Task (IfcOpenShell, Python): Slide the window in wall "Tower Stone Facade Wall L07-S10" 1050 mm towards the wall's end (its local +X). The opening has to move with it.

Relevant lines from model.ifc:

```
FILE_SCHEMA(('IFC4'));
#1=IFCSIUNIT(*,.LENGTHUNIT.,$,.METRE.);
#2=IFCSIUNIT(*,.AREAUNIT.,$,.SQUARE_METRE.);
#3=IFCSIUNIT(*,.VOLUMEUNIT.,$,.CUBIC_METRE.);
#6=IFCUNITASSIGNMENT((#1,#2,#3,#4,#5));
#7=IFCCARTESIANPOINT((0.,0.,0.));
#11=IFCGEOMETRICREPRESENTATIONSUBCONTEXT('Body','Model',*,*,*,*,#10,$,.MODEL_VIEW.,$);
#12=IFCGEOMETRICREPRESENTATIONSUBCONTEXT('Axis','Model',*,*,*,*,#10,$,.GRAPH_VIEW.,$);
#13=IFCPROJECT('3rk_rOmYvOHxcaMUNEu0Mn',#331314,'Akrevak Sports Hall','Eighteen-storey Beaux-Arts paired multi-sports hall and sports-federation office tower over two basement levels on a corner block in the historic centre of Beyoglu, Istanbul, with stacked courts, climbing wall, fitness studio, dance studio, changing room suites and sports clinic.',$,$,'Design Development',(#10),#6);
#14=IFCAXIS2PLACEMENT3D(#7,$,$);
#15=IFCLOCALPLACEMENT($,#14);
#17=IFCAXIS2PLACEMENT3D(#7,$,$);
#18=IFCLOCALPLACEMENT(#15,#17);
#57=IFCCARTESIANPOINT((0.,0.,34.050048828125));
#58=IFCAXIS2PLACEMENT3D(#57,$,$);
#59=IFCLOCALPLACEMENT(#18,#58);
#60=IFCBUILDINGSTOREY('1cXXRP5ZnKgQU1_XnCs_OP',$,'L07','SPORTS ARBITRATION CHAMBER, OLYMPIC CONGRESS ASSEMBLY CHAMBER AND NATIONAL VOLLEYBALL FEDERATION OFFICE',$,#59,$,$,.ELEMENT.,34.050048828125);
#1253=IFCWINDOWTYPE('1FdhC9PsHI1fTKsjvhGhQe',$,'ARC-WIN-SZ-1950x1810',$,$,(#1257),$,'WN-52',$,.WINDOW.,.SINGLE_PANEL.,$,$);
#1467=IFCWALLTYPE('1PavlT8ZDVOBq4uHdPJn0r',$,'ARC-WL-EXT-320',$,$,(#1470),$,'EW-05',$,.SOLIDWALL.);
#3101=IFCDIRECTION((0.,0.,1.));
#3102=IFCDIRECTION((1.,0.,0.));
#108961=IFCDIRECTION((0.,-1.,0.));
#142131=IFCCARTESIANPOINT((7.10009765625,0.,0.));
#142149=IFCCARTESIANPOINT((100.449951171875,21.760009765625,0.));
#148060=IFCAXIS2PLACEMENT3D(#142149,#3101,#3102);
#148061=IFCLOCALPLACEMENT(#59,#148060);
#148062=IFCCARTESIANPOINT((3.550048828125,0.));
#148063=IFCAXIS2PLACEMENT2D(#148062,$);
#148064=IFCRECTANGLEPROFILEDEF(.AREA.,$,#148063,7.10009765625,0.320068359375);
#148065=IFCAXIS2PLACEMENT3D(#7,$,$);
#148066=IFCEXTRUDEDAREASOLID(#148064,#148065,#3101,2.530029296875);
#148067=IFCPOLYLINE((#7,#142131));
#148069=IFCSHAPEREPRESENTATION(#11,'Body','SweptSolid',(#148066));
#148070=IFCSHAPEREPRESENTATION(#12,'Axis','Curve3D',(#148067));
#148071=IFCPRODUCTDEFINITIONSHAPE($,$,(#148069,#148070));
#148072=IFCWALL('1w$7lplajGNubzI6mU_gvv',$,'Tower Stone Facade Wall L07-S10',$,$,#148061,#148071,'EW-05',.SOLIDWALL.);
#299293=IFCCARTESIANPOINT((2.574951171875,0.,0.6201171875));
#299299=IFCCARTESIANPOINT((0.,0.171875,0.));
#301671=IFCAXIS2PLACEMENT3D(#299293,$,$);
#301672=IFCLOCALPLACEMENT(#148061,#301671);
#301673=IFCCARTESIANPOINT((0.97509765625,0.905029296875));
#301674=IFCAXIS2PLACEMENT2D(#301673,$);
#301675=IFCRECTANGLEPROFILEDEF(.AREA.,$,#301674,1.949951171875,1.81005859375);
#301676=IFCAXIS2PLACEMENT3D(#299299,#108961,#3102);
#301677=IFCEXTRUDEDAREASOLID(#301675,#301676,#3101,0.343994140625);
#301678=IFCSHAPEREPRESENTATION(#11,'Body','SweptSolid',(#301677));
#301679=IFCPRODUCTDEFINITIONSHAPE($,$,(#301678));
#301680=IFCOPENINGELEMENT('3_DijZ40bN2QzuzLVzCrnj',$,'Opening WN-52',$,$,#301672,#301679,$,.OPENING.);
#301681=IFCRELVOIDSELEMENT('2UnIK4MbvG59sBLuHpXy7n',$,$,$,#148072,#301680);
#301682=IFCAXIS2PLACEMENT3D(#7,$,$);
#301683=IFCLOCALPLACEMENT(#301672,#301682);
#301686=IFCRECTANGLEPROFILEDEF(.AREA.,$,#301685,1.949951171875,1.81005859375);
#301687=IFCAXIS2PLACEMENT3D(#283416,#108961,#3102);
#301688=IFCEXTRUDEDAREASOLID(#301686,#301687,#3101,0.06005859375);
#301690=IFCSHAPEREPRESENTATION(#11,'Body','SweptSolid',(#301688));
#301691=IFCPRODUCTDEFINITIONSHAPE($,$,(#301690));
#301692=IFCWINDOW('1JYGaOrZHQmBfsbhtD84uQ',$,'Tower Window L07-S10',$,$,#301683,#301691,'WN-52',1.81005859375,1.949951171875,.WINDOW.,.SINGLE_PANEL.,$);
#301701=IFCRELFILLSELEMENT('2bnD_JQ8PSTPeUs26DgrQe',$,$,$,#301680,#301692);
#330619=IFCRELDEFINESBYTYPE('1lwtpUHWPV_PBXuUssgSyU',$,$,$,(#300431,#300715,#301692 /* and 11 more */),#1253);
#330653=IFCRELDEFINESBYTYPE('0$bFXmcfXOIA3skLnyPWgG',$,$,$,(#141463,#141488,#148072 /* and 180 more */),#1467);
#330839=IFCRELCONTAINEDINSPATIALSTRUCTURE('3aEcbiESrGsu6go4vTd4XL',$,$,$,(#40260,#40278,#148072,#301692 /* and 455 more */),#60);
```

```python
import ifcopenshell
import ifcopenshell.api.geometry
import ifcopenshell.util.placement

model = ifcopenshell.open("model.ifc")

window = model.by_guid("1JYGaOrZHQmBfsbhtD84uQ")
opening = window.FillsVoids[0].RelatingOpeningElement
wall = opening.VoidsElements[0].RelatingBuildingElement

wall_matrix = ifcopenshell.util.placement.get_local_placement(wall.ObjectPlacement)
shift = wall_matrix[:3, 0] * 1.05
before = ifcopenshell.util.placement.get_local_placement(window.ObjectPlacement)[:3, 3].copy()

# The window is placed relative to its opening, so it follows when the opening moves.
matrix = ifcopenshell.util.placement.get_local_placement(opening.ObjectPlacement)
matrix[:3, 3] += shift
ifcopenshell.api.geometry.edit_object_placement(
    model, product=opening, matrix=matrix, is_si=False, should_transform_children=True
)

after = ifcopenshell.util.placement.get_local_placement(window.ObjectPlacement)[:3, 3]
print("window moved by", (after - before).round(3) + 0.0)

model.write("model_v2.ifc")
```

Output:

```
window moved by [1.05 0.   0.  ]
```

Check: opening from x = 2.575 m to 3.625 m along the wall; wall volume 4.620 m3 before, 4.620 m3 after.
